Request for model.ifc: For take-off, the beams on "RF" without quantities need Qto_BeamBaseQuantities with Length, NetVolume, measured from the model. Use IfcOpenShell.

First a look at what the model holds.

```python
import ifcopenshell
import ifcopenshell.util.element
import ifcopenshell.util.unit

model = ifcopenshell.open("model.ifc")
print(model.schema)
for unit_type in ("LENGTHUNIT", "AREAUNIT", "VOLUMEUNIT"):
    print(unit_type, ifcopenshell.util.unit.calculate_unit_scale(model, unit_type))
storey = next(s for s in model.by_type("IfcBuildingStorey") if s.Name == "RF")
beams = [e for e in ifcopenshell.util.element.get_decomposition(storey) if e.is_a("IfcBeam")]
for e in sorted(beams, key=lambda e: e.id()):
    print(e.id(), e.is_a(), e.Name, list(ifcopenshell.util.element.get_psets(e, qtos_only=True)), sep=" | ")
```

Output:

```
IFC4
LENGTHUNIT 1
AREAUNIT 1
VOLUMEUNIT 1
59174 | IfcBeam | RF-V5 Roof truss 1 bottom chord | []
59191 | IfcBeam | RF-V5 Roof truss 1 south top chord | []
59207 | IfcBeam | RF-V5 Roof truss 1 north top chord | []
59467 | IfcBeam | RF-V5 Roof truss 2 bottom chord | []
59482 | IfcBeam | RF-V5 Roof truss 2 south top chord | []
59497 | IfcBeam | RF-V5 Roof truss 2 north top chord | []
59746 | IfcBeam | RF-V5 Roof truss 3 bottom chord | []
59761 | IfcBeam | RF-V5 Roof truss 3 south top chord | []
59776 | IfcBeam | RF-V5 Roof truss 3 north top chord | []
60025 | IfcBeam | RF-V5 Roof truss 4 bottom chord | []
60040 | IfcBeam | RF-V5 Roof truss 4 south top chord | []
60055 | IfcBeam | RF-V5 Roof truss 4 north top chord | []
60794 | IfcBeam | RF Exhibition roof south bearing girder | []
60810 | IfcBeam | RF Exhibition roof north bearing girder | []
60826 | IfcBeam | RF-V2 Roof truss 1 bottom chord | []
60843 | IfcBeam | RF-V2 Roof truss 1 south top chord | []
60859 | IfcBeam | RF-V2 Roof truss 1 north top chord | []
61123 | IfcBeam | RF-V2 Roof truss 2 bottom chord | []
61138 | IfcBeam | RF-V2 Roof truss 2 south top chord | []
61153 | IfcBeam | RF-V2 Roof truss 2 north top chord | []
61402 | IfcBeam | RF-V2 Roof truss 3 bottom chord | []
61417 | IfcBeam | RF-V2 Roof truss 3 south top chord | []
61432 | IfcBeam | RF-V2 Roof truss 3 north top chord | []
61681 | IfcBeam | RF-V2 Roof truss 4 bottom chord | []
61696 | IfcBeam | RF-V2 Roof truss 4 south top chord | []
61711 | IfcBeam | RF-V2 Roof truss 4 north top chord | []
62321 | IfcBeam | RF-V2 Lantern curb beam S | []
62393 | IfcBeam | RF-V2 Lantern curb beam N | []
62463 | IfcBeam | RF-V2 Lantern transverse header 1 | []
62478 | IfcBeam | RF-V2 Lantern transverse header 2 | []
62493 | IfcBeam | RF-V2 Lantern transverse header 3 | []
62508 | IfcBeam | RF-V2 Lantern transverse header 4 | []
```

```python
import ifcopenshell
import ifcopenshell.api.pset
import ifcopenshell.geom
import ifcopenshell.util.element
import ifcopenshell.util.shape
import ifcopenshell.util.unit

model = ifcopenshell.open("model.ifc")
unit_scale = ifcopenshell.util.unit.calculate_unit_scale(model)
volume_scale = ifcopenshell.util.unit.calculate_unit_scale(model, "VOLUMEUNIT")
settings = ifcopenshell.geom.settings()

storey = next(s for s in model.by_type("IfcBuildingStorey") if s.Name == "RF")
beams = [e for e in ifcopenshell.util.element.get_decomposition(storey) if e.is_a("IfcBeam")]

for e in sorted(beams, key=lambda e: e.id()):
    if ifcopenshell.util.element.get_psets(e, qtos_only=True, should_inherit=False):
        continue
    # Geometry comes back in metres, in the element's own axes.
    shape = ifcopenshell.geom.create_shape(settings, e)
    values = {
        "Length": ifcopenshell.util.shape.get_max_xyz(shape.geometry) / unit_scale,
        "NetVolume": ifcopenshell.util.shape.get_volume(shape.geometry) / volume_scale,
    }
    qto = ifcopenshell.api.pset.add_qto(model, product=e, name="Qto_BeamBaseQuantities")
    ifcopenshell.api.pset.edit_qto(model, qto=qto, properties=values)
    print(e.id(), {k: round(v, 3) for k, v in values.items()})

model.write("model_updated.ifc")
```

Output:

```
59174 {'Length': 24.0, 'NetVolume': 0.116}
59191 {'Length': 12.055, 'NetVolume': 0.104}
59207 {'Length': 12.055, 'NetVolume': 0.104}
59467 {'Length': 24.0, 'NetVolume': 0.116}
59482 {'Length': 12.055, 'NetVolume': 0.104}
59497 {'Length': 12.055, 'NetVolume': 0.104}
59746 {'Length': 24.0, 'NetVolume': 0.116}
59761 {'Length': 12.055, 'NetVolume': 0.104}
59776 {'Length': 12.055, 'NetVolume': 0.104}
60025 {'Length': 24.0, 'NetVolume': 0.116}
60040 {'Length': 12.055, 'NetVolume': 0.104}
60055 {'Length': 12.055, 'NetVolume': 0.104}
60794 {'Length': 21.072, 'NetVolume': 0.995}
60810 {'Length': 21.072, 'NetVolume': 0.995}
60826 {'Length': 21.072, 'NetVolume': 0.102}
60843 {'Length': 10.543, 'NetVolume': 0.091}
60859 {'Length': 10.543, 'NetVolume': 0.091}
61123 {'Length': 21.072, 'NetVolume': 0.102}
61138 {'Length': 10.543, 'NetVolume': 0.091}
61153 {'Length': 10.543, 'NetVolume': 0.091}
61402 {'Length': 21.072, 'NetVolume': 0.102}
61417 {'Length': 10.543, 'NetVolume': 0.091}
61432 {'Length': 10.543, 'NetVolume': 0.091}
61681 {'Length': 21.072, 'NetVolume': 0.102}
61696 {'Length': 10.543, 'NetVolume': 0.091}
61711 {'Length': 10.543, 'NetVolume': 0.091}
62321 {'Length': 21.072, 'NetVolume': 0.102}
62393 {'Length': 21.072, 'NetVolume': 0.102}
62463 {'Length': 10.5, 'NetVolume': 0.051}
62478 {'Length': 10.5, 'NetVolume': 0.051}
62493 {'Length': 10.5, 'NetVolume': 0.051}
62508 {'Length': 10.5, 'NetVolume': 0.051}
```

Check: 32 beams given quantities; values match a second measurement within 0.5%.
